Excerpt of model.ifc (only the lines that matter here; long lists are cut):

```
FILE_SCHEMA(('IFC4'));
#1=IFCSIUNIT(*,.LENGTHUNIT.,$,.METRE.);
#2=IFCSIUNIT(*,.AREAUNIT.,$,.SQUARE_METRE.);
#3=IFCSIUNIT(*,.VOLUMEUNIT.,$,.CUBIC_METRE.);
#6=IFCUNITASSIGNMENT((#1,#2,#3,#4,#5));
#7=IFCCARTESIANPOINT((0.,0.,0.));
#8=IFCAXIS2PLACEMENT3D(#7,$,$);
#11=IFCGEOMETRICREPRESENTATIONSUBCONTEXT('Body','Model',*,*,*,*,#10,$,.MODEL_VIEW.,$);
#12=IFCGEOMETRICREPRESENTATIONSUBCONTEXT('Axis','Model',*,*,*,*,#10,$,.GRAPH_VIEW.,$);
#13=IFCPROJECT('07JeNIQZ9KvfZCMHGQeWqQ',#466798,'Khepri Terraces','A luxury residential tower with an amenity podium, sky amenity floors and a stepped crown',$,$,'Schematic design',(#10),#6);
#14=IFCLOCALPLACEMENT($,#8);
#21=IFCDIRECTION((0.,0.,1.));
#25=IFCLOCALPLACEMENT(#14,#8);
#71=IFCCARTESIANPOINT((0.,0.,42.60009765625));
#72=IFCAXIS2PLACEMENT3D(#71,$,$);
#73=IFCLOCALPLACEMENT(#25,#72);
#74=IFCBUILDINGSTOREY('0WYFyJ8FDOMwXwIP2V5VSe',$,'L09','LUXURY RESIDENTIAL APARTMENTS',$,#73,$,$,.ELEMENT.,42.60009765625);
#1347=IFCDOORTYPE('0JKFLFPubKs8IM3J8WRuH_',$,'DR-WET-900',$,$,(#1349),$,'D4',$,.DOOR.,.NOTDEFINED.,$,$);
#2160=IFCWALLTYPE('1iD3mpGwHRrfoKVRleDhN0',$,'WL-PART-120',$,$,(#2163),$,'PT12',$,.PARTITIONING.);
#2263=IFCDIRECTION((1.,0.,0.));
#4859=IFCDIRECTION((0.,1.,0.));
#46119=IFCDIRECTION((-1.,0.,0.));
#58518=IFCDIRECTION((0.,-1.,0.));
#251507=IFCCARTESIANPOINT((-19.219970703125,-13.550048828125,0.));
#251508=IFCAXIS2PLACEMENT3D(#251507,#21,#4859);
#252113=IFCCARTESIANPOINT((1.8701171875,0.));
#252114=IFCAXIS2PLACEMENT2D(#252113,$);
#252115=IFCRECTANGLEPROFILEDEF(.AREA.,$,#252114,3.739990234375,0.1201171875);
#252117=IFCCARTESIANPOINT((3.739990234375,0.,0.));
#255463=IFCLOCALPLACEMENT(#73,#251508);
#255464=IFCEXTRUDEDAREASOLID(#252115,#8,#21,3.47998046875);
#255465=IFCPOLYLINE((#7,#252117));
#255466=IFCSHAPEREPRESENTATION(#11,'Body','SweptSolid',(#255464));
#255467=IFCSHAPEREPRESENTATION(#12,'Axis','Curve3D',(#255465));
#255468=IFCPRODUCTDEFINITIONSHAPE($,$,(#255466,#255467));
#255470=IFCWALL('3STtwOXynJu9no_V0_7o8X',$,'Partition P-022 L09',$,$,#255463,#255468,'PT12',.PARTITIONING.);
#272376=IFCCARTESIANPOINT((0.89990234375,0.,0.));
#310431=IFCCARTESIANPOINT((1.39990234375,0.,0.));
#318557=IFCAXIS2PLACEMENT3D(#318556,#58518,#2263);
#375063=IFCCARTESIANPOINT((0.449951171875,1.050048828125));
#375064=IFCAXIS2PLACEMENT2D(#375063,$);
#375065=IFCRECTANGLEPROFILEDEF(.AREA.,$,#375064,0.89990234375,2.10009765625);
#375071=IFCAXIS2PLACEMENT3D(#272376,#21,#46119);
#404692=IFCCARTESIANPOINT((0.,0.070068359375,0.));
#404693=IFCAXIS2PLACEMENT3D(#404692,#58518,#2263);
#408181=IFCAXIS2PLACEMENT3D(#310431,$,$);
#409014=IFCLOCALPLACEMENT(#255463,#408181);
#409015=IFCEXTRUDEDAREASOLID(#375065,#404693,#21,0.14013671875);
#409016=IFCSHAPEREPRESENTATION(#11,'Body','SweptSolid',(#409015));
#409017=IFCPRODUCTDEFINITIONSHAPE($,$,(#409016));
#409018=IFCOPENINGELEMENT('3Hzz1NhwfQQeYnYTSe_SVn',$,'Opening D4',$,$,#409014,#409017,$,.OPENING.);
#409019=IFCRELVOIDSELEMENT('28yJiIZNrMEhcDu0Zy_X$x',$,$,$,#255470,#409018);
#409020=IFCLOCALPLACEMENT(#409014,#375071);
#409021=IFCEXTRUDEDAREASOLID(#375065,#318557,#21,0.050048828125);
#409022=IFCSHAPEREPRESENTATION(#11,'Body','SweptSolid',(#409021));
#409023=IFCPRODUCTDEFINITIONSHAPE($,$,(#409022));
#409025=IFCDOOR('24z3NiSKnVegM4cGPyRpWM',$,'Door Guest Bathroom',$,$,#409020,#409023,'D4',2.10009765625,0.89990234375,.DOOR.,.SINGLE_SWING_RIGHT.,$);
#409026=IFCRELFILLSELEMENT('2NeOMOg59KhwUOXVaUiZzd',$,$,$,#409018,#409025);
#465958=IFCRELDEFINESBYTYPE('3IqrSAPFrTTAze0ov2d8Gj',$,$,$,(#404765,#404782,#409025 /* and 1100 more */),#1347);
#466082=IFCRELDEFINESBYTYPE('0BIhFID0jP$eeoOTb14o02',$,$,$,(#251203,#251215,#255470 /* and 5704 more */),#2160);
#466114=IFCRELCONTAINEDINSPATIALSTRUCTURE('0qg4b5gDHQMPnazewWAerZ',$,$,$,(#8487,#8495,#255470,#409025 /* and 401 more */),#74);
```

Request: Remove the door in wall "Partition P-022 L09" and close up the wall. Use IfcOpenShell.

```python
import ifcopenshell
import ifcopenshell.api.feature
import ifcopenshell.api.root
import ifcopenshell.geom
import ifcopenshell.util.shape

model = ifcopenshell.open("model.ifc")
settings = ifcopenshell.geom.settings()


def volume(element):
    """Net volume in cubic metres, openings subtracted."""
    shape = ifcopenshell.geom.create_shape(settings, element)
    return ifcopenshell.util.shape.get_volume(shape.geometry)


door = model.by_id(409025)
opening = door.FillsVoids[0].RelatingOpeningElement
wall = opening.VoidsElements[0].RelatingBuildingElement
before = volume(wall)

ifcopenshell.api.root.remove_product(model, product=door)
ifcopenshell.api.feature.remove_feature(model, feature=opening)

after = volume(wall)

print(f"wall volume {before:.3f} -> {after:.3f} m3")

model.write("model_edited.ifc")
```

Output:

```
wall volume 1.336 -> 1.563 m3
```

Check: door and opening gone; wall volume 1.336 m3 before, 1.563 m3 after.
